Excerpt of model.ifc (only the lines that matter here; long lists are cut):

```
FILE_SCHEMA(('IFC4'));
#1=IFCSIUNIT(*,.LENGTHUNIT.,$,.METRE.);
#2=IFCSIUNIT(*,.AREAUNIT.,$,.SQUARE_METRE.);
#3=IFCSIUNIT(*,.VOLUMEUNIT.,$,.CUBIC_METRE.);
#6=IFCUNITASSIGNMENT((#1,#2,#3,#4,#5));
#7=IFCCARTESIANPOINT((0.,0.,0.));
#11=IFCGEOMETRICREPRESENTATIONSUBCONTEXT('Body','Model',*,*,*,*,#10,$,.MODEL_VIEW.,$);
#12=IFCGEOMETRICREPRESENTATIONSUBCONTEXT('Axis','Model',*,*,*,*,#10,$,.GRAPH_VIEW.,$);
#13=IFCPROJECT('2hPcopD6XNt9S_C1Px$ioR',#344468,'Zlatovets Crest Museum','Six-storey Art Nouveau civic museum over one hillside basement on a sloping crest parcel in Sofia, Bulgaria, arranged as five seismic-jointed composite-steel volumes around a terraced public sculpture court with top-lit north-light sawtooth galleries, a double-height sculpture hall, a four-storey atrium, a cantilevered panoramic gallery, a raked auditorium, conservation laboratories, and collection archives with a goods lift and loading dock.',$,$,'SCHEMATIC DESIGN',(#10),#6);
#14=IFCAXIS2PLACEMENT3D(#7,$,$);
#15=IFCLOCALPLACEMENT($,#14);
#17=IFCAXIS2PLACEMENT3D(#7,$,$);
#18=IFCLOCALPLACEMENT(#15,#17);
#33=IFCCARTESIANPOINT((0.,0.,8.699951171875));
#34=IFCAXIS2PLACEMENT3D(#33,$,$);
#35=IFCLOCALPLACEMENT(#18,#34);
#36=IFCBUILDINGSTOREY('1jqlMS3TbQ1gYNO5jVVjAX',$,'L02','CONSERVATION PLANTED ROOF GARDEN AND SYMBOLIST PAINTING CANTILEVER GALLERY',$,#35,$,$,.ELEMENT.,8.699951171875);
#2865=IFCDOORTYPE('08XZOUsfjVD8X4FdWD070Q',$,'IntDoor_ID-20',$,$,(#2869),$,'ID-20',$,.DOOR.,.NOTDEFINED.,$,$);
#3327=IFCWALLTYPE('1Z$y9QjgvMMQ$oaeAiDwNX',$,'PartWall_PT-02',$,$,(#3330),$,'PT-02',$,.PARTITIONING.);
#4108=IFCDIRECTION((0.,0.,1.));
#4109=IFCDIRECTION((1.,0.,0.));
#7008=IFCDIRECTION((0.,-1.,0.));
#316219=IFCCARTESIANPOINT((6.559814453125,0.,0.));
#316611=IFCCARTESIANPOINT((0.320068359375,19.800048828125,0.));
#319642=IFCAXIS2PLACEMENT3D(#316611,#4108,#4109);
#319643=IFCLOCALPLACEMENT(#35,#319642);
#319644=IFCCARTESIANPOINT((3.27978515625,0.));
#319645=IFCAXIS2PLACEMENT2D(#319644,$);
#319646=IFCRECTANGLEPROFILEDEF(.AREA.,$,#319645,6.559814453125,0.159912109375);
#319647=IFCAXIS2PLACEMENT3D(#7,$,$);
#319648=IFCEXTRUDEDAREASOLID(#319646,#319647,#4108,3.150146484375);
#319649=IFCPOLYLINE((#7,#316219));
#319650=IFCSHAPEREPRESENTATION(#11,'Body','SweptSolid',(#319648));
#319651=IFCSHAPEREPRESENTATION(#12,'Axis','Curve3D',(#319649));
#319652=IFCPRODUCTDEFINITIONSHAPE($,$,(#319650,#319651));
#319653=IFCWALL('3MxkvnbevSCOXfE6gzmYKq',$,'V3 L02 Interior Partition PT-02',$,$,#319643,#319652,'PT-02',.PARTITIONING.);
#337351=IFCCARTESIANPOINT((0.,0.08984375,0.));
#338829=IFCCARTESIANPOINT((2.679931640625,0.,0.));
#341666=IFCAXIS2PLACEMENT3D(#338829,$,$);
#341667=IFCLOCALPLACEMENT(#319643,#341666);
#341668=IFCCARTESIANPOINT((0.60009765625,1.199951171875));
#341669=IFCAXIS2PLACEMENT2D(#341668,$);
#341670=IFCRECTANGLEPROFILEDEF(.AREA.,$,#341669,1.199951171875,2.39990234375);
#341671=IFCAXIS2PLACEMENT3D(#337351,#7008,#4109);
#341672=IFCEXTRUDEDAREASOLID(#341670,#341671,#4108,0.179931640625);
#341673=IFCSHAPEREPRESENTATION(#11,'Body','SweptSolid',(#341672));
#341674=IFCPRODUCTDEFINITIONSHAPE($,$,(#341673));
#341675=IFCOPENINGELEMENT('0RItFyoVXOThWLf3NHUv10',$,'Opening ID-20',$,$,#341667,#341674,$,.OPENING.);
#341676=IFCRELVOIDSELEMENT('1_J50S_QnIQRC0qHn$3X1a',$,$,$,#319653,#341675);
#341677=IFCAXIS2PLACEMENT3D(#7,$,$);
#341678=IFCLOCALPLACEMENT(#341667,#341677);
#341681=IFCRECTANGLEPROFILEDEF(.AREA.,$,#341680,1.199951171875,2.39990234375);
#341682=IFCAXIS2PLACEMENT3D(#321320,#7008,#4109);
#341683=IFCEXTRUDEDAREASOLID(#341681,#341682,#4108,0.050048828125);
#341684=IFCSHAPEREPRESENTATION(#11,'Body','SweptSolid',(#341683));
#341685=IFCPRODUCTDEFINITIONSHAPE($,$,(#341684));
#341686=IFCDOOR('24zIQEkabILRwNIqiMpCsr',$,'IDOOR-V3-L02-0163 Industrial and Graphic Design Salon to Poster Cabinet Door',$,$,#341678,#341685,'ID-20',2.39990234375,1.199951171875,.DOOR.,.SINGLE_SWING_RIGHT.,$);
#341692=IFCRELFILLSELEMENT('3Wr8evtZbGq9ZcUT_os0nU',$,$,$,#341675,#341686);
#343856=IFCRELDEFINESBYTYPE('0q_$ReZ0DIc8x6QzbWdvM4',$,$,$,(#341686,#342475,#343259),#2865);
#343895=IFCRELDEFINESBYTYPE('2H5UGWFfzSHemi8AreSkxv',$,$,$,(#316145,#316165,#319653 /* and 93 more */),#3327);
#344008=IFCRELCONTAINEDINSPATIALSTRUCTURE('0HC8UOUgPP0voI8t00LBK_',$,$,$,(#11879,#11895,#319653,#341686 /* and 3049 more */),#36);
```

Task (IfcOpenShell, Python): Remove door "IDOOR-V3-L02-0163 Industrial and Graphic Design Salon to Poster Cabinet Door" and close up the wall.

```python
import ifcopenshell
import ifcopenshell.api.feature
import ifcopenshell.api.root
import ifcopenshell.geom
import ifcopenshell.util.shape

model = ifcopenshell.open("model.ifc")
settings = ifcopenshell.geom.settings()


def volume(element):
    """Net volume in cubic metres, openings subtracted."""
    shape = ifcopenshell.geom.create_shape(settings, element)
    return ifcopenshell.util.shape.get_volume(shape.geometry)


door = model.by_guid("24zIQEkabILRwNIqiMpCsr")
opening = door.FillsVoids[0].RelatingOpeningElement
wall = opening.VoidsElements[0].RelatingBuildingElement
before = volume(wall)

ifcopenshell.api.root.remove_product(model, product=door)
ifcopenshell.api.feature.remove_feature(model, feature=opening)

after = volume(wall)

print(f"wall volume {before:.3f} -> {after:.3f} m3")

model.write("model-out.ifc")
```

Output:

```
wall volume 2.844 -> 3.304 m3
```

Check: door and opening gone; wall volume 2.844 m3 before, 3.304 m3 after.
